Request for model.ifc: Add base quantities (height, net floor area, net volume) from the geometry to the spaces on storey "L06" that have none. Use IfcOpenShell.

First a look at what the model holds.

```python
import ifcopenshell
import ifcopenshell.util.element
import ifcopenshell.util.unit

model = ifcopenshell.open("model.ifc")
print(model.schema)
for unit_type in ("LENGTHUNIT", "AREAUNIT", "VOLUMEUNIT"):
    print(unit_type, ifcopenshell.util.unit.calculate_unit_scale(model, unit_type))
storey = next(s for s in model.by_type("IfcBuildingStorey") if s.Name == "L06")
spaces = [e for e in ifcopenshell.util.element.get_decomposition(storey) if e.is_a("IfcSpace")]
for e in sorted(spaces, key=lambda e: e.id()):
    print(e.id(), e.is_a(), e.Name, list(ifcopenshell.util.element.get_psets(e, qtos_only=True)), sep=" | ")
```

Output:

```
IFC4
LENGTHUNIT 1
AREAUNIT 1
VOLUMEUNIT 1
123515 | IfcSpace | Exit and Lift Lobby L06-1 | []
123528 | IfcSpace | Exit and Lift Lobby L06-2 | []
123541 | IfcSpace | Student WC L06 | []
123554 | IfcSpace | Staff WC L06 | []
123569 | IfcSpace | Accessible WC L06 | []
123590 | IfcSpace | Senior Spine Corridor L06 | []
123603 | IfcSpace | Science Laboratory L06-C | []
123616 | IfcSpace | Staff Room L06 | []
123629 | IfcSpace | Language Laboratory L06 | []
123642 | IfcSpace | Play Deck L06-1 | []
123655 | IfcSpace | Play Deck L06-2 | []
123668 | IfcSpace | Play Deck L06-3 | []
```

```python
import ifcopenshell
import ifcopenshell.api.pset
import ifcopenshell.geom
import ifcopenshell.util.element
import ifcopenshell.util.shape
import ifcopenshell.util.unit

model = ifcopenshell.open("model.ifc")
unit_scale = ifcopenshell.util.unit.calculate_unit_scale(model)
area_scale = ifcopenshell.util.unit.calculate_unit_scale(model, "AREAUNIT")
volume_scale = ifcopenshell.util.unit.calculate_unit_scale(model, "VOLUMEUNIT")
settings = ifcopenshell.geom.settings()

storey = next(s for s in model.by_type("IfcBuildingStorey") if s.Name == "L06")
spaces = [e for e in ifcopenshell.util.element.get_decomposition(storey) if e.is_a("IfcSpace")]

for e in sorted(spaces, key=lambda e: e.id()):
    if ifcopenshell.util.element.get_psets(e, qtos_only=True, should_inherit=False):
        continue
    # Geometry comes back in metres, in the element's own axes.
    shape = ifcopenshell.geom.create_shape(settings, e)
    values = {
        "Height": ifcopenshell.util.shape.get_z(shape.geometry) / unit_scale,
        "NetFloorArea": ifcopenshell.util.shape.get_footprint_area(shape.geometry) / area_scale,
        "NetVolume": ifcopenshell.util.shape.get_volume(shape.geometry) / volume_scale,
    }
    qto = ifcopenshell.api.pset.add_qto(model, product=e, name="Qto_SpaceBaseQuantities")
    ifcopenshell.api.pset.edit_qto(model, qto=qto, properties=values)
    print(e.id(), {k: round(v, 3) for k, v in values.items()})

model.write("model_edited.ifc")
```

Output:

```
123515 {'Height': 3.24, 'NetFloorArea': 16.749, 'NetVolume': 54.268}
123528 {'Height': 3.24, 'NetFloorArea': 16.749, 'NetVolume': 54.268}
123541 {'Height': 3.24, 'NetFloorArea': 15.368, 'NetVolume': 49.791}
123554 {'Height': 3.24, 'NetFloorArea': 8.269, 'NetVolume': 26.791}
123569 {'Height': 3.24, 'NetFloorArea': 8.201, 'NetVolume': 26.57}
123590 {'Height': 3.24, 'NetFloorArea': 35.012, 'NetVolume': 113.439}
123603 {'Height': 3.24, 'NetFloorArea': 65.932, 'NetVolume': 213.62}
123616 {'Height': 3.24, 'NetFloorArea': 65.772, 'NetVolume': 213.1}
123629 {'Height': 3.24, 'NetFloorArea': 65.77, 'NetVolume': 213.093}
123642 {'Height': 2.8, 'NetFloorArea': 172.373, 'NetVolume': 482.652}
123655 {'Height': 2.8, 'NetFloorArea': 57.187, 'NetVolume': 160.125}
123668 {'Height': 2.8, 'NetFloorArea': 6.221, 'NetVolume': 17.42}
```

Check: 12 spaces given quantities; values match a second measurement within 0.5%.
